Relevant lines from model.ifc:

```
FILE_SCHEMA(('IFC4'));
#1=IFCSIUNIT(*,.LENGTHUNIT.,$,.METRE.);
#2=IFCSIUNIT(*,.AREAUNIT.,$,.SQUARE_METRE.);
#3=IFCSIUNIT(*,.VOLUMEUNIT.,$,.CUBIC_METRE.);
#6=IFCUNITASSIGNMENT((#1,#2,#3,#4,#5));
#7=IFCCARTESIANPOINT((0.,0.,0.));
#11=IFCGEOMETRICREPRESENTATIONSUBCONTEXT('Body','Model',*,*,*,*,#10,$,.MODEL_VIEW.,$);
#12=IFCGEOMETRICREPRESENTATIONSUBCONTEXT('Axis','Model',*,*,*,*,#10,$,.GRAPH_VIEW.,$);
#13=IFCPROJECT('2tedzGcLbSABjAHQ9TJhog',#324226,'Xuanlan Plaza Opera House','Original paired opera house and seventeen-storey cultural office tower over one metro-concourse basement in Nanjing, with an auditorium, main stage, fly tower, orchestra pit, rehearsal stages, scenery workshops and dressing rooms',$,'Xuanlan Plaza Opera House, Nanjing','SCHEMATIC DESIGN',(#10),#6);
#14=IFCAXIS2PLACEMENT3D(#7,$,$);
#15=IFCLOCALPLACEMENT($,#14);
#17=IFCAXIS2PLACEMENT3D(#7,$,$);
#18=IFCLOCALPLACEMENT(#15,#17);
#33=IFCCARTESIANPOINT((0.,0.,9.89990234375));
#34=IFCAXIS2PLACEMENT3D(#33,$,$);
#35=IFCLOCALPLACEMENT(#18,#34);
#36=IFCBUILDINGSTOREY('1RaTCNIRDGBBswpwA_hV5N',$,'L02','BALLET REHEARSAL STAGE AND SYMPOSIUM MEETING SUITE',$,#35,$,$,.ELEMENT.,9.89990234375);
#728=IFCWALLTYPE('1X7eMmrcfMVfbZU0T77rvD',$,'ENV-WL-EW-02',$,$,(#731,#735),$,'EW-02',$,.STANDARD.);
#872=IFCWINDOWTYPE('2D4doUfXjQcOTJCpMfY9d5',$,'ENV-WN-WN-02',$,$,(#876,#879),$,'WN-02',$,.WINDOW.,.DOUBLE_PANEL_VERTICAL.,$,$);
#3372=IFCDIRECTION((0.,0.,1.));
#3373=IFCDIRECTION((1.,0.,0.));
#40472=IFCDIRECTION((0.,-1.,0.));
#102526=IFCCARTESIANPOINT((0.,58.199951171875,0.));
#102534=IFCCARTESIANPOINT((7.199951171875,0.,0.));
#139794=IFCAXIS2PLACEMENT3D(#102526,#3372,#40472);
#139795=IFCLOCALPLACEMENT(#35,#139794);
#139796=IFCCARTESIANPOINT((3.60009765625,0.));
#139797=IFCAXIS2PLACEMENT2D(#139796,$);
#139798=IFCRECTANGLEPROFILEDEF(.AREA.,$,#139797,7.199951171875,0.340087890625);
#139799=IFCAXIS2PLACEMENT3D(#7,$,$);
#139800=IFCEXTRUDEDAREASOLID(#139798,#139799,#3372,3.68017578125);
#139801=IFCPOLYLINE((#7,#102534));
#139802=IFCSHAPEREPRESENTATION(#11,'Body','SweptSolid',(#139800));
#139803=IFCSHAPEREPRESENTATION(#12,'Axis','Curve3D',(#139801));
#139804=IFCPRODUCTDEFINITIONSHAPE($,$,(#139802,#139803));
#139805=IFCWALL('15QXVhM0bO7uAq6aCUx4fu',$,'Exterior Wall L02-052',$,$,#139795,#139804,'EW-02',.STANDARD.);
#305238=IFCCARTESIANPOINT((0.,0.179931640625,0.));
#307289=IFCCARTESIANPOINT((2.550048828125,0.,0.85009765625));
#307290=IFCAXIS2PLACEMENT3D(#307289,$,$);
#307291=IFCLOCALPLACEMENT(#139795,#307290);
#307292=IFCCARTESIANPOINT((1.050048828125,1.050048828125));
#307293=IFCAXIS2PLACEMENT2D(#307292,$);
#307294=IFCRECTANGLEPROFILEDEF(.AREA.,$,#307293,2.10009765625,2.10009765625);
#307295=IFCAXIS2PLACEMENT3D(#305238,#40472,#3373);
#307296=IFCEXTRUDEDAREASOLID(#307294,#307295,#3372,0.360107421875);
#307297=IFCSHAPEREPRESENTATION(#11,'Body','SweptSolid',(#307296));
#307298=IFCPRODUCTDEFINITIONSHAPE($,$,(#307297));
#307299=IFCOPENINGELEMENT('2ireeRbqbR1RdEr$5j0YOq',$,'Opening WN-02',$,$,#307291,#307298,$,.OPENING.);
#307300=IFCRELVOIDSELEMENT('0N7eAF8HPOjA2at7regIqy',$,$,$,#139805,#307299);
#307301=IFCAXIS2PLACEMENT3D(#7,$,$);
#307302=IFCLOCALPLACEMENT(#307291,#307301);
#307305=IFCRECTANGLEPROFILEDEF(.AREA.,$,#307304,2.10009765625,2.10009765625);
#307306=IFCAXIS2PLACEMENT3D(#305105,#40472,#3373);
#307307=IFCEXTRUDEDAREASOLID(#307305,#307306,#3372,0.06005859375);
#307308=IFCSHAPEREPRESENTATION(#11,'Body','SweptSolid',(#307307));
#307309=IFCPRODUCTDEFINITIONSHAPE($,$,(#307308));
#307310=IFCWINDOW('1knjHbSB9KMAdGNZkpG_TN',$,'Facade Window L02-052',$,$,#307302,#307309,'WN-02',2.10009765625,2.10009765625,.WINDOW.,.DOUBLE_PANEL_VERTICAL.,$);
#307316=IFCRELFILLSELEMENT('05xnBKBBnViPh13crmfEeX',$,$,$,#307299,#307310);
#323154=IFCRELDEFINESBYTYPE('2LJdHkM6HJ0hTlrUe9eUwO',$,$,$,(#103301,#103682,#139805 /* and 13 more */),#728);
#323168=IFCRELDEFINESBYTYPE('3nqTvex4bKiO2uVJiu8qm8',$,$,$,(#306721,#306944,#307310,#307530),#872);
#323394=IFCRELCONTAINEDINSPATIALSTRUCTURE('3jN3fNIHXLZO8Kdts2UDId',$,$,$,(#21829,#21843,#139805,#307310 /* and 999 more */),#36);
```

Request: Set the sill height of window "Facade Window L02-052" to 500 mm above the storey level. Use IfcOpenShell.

```python
import numpy as np
import ifcopenshell
import ifcopenshell.api.geometry
import ifcopenshell.geom
import ifcopenshell.util.element
import ifcopenshell.util.placement
import ifcopenshell.util.shape
import ifcopenshell.util.unit

model = ifcopenshell.open("model.ifc")
unit_scale = ifcopenshell.util.unit.calculate_unit_scale(model)

window = model.by_id(307310)
opening = window.FillsVoids[0].RelatingOpeningElement
storey = ifcopenshell.util.element.get_container(window, ifc_class="IfcBuildingStorey")
level = ifcopenshell.util.placement.get_local_placement(storey.ObjectPlacement)[2, 3]

# The opening's origin need not be at the sill, so measure its lowest point.
shape = ifcopenshell.geom.create_shape(ifcopenshell.geom.settings(), opening)
bottom = ifcopenshell.util.shape.get_shape_bottom_elevation(shape, shape.geometry) / unit_scale
dz = level + 0.5 - bottom

shift = np.array([0.0, 0.0, dz])
# The window is placed relative to its opening, so it follows when the opening moves.
matrix = ifcopenshell.util.placement.get_local_placement(opening.ObjectPlacement)
matrix[:3, 3] += shift
ifcopenshell.api.geometry.edit_object_placement(
    model, product=opening, matrix=matrix, is_si=False, should_transform_children=True
)

print(f"moved by {dz * unit_scale:+.3f} m")

model.write("model_updated.ifc")
```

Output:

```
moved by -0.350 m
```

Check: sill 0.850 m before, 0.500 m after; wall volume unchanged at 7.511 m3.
